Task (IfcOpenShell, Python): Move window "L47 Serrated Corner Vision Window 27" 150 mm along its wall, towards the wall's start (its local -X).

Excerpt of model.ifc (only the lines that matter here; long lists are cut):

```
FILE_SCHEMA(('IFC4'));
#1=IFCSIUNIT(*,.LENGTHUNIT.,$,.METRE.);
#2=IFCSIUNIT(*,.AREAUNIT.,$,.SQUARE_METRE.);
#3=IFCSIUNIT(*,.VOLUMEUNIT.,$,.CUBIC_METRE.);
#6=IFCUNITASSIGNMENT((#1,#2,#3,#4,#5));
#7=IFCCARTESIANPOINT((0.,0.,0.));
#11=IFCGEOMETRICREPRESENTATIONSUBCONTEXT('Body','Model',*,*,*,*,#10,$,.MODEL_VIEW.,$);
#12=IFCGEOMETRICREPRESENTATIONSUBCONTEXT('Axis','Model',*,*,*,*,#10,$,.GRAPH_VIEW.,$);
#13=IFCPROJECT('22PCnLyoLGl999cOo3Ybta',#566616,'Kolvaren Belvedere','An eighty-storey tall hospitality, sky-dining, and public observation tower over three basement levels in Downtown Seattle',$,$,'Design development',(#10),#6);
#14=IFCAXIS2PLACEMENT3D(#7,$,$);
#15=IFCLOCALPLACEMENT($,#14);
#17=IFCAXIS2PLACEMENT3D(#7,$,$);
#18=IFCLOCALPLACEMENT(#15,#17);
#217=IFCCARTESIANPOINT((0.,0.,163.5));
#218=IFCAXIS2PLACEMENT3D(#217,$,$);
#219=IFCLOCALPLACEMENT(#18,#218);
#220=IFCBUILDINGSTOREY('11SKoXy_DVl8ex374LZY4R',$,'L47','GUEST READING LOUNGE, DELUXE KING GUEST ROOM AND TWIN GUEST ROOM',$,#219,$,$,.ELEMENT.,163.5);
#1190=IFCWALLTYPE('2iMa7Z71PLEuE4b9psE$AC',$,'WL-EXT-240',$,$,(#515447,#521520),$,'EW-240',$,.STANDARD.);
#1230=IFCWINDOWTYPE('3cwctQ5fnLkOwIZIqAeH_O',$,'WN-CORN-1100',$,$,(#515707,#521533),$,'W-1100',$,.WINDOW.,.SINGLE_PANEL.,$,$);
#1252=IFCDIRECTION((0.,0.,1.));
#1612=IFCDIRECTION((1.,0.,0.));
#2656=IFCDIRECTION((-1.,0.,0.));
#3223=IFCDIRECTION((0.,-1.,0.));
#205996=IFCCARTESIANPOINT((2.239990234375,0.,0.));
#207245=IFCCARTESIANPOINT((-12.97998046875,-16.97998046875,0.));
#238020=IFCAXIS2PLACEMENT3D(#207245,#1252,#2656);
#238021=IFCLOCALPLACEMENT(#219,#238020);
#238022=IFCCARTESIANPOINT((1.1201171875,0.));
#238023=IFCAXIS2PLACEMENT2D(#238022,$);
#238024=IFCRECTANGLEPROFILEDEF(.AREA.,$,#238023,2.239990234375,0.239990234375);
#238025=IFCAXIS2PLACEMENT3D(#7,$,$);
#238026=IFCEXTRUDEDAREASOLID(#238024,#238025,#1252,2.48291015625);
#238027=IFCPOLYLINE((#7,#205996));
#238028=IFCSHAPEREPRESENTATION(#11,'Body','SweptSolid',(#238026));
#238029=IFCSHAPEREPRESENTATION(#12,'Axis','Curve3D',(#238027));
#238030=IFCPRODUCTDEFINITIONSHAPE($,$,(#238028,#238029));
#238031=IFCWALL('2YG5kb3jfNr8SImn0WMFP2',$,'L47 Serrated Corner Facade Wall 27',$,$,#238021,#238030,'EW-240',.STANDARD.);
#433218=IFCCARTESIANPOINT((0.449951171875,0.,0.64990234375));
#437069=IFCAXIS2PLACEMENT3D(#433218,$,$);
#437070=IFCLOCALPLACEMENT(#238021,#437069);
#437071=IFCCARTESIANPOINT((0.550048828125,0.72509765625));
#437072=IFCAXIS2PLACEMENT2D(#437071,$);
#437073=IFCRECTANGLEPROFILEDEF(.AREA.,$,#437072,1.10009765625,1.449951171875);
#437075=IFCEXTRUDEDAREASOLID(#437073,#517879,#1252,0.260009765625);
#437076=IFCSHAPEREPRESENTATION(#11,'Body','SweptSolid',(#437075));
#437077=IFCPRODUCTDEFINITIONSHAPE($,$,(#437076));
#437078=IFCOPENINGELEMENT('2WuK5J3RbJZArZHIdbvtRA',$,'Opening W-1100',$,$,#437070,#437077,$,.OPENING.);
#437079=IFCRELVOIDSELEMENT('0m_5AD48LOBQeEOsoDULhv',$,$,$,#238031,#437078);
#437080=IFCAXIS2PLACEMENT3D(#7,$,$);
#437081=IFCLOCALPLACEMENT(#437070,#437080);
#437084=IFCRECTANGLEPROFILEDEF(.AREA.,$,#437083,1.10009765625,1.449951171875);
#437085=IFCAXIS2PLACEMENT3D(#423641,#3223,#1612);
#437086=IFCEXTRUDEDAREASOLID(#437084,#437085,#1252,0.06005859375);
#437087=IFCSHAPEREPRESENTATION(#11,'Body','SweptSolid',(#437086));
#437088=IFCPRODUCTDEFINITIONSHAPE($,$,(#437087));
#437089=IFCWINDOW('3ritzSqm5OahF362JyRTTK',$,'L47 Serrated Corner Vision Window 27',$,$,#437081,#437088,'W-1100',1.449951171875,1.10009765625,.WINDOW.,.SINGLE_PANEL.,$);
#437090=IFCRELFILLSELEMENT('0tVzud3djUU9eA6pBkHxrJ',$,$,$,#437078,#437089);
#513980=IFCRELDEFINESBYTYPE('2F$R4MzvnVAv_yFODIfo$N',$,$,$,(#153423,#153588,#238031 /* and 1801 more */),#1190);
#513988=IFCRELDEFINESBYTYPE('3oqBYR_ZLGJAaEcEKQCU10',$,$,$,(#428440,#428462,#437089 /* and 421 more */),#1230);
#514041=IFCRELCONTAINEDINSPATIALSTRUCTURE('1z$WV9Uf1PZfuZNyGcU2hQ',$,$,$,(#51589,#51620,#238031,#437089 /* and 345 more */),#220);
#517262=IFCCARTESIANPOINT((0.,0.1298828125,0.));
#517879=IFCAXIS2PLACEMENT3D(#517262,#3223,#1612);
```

```python
import ifcopenshell
import ifcopenshell.api.geometry
import ifcopenshell.util.placement
import ifcopenshell.util.unit

model = ifcopenshell.open("model.ifc")
unit_scale = ifcopenshell.util.unit.calculate_unit_scale(model)

window = model.by_guid("3ritzSqm5OahF362JyRTTK")
opening = window.FillsVoids[0].RelatingOpeningElement
wall = opening.VoidsElements[0].RelatingBuildingElement

wall_matrix = ifcopenshell.util.placement.get_local_placement(wall.ObjectPlacement)
shift = wall_matrix[:3, 0] * -0.15 / unit_scale
before = ifcopenshell.util.placement.get_local_placement(window.ObjectPlacement)[:3, 3].copy()

# The window is placed relative to its opening, so it follows when the opening moves.
matrix = ifcopenshell.util.placement.get_local_placement(opening.ObjectPlacement)
matrix[:3, 3] += shift
ifcopenshell.api.geometry.edit_object_placement(
    model, product=opening, matrix=matrix, is_si=False, should_transform_children=True
)

after = ifcopenshell.util.placement.get_local_placement(window.ObjectPlacement)[:3, 3]
print("window moved by", (after - before).round(3) + 0.0)

model.write("model_updated.ifc")
```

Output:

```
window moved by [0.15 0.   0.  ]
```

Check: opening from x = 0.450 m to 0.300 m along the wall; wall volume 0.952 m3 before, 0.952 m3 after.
